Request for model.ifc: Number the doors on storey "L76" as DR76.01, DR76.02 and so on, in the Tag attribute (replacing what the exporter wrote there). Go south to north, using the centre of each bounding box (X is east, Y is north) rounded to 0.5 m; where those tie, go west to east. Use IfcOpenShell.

First a look at what the model holds.

```python
import ifcopenshell
import ifcopenshell.util.element
import ifcopenshell.util.placement

model = ifcopenshell.open("model.ifc")
print(model.schema)
storey = next(s for s in model.by_type("IfcBuildingStorey") if s.Name == "L76")
doors = [e for e in ifcopenshell.util.element.get_decomposition(storey) if e.is_a("IfcDoor")]
for e in sorted(doors, key=lambda e: e.id()):
    origin = ifcopenshell.util.placement.get_local_placement(e.ObjectPlacement)[:3, 3]
    print(e.id(), e.Tag, e.Name, origin.round(2) + 0.0, sep=" | ")
```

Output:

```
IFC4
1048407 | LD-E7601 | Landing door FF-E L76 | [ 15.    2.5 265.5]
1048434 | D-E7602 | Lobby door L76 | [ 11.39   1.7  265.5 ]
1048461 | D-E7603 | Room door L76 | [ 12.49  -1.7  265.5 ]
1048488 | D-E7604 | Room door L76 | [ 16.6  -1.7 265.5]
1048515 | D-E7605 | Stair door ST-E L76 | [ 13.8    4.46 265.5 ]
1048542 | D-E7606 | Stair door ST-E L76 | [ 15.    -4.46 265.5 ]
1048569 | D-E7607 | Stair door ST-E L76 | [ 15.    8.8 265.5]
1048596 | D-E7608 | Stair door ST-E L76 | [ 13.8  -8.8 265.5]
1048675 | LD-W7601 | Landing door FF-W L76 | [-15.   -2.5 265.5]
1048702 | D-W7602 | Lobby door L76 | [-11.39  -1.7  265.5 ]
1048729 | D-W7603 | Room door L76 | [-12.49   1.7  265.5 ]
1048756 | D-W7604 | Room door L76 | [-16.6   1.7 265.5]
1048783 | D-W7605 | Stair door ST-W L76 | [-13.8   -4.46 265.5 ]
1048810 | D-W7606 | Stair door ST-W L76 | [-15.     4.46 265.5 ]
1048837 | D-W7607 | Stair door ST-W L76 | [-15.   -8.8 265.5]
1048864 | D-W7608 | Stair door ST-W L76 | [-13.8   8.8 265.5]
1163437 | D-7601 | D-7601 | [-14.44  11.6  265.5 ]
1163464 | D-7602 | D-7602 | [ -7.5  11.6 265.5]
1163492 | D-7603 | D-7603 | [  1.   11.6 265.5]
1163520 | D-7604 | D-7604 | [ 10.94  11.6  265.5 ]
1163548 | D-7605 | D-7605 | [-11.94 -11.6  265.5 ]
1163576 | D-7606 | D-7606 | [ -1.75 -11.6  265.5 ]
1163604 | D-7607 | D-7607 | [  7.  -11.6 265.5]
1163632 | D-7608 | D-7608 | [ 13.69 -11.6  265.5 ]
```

```python
import ifcopenshell
import ifcopenshell.geom
import ifcopenshell.util.element
import ifcopenshell.util.shape

model = ifcopenshell.open("model.ifc")
settings = ifcopenshell.geom.settings()
settings.set("use-world-coords", True)


def centre(element):
    shape = ifcopenshell.geom.create_shape(settings, element)
    return ifcopenshell.util.shape.get_bbox_centroid(shape.geometry)


storey = next(s for s in model.by_type("IfcBuildingStorey") if s.Name == "L76")
doors = [e for e in ifcopenshell.util.element.get_decomposition(storey) if e.is_a("IfcDoor")]

# Insertion points can sit at a corner or the storey origin, so sort by the geometry (in metres).
centres = {e: centre(e) for e in doors}
doors.sort(key=lambda e: (round(centres[e][1] / 0.5), centres[e][0]))

for i, e in enumerate(doors, start=1):
    number = f"DR76.{i:02d}"
    e.Tag = number
    print(e.id(), number)

model.write("model_v2.ifc")
```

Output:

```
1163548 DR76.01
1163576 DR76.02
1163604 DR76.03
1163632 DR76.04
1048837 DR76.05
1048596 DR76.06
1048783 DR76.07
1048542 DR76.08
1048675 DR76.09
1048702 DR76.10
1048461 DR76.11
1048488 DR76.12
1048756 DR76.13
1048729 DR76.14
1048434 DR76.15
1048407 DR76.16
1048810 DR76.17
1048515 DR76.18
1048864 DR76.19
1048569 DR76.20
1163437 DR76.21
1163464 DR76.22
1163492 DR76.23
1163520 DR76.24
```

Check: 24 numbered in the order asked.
